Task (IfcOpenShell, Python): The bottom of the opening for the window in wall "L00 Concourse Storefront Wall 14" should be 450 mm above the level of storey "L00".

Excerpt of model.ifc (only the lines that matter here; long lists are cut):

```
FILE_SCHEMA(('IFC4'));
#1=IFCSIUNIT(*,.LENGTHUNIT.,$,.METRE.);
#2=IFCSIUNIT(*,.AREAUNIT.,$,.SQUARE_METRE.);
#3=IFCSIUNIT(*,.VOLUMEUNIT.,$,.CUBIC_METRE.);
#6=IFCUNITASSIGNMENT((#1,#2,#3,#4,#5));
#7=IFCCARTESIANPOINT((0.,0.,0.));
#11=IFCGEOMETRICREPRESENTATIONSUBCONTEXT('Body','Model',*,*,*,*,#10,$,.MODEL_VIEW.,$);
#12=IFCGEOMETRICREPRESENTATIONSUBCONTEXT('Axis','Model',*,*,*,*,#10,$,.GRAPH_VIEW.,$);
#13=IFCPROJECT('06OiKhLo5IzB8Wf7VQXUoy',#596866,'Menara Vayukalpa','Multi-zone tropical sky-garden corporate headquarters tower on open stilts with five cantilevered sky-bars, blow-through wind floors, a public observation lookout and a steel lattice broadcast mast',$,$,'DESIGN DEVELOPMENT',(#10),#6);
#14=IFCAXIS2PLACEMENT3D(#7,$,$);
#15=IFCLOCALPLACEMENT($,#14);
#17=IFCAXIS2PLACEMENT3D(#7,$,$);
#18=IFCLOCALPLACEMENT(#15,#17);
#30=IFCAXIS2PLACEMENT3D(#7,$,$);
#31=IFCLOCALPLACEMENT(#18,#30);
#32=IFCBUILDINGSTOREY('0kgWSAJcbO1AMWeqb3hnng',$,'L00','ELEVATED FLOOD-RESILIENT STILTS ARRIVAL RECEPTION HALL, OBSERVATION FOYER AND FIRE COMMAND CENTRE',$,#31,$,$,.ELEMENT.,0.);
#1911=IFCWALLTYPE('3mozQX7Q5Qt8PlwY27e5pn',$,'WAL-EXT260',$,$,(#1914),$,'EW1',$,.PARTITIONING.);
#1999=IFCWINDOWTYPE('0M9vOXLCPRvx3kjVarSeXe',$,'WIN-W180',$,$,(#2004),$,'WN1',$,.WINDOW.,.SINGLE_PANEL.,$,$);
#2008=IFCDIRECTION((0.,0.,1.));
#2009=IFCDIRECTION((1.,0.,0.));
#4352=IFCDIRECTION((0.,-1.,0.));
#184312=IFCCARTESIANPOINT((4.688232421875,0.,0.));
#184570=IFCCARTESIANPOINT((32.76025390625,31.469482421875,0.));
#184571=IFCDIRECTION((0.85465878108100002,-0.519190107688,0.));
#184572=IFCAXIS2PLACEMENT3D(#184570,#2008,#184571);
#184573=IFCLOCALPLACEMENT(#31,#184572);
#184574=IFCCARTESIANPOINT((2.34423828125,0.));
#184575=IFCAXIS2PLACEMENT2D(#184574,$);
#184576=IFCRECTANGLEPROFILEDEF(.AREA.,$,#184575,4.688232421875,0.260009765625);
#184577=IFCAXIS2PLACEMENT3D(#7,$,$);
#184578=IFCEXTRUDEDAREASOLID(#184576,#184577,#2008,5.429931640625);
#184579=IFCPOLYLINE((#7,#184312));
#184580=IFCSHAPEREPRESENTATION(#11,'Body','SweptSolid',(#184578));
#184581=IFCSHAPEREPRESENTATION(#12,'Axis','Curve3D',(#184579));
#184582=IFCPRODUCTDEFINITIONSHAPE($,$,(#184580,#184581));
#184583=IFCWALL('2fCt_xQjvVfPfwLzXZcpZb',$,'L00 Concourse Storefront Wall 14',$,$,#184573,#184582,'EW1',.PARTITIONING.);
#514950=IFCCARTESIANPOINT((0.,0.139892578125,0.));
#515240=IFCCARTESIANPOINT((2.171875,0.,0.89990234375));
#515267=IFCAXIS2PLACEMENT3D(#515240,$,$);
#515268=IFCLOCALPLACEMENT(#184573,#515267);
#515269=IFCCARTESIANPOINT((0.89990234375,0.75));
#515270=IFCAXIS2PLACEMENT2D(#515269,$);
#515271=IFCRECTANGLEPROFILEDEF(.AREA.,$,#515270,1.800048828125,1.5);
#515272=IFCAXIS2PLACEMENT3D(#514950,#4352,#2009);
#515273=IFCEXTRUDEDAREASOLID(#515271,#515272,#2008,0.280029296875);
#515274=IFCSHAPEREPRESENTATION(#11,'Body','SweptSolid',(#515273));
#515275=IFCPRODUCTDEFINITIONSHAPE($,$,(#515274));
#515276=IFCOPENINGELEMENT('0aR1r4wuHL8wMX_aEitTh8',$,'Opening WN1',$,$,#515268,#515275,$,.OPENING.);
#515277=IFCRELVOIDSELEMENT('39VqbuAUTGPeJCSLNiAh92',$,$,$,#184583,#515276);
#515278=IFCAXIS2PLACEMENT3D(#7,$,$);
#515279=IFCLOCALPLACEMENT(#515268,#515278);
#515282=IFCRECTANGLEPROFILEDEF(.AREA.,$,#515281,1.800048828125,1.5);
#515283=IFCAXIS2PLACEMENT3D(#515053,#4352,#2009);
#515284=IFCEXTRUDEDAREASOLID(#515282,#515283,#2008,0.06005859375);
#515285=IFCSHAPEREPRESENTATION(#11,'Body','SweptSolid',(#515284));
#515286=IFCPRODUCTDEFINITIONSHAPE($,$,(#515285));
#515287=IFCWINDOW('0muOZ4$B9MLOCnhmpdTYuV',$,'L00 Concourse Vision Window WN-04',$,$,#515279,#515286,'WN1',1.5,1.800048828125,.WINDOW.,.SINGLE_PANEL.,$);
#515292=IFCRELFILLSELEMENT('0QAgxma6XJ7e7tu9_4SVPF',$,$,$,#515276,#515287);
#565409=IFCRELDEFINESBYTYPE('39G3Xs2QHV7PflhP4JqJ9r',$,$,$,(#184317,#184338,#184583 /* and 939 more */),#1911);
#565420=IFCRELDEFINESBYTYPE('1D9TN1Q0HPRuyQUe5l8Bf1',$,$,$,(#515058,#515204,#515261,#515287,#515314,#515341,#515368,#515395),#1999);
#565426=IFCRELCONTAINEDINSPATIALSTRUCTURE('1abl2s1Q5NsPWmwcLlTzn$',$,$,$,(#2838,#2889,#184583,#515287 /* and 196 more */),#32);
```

```python
import numpy as np
import ifcopenshell
import ifcopenshell.api.geometry
import ifcopenshell.geom
import ifcopenshell.util.element
import ifcopenshell.util.placement
import ifcopenshell.util.shape
import ifcopenshell.util.unit

model = ifcopenshell.open("model.ifc")
unit_scale = ifcopenshell.util.unit.calculate_unit_scale(model)

window = model.by_guid("0muOZ4$B9MLOCnhmpdTYuV")
opening = window.FillsVoids[0].RelatingOpeningElement
storey = ifcopenshell.util.element.get_container(window, ifc_class="IfcBuildingStorey")
level = ifcopenshell.util.placement.get_local_placement(storey.ObjectPlacement)[2, 3]

# The opening's origin need not be at the sill, so measure its lowest point.
shape = ifcopenshell.geom.create_shape(ifcopenshell.geom.settings(), opening)
bottom = ifcopenshell.util.shape.get_shape_bottom_elevation(shape, shape.geometry) / unit_scale
dz = level + 0.45 - bottom

shift = np.array([0.0, 0.0, dz])
# The window is placed relative to its opening, so it follows when the opening moves.
matrix = ifcopenshell.util.placement.get_local_placement(opening.ObjectPlacement)
matrix[:3, 3] += shift
ifcopenshell.api.geometry.edit_object_placement(
    model, product=opening, matrix=matrix, is_si=False, should_transform_children=True
)

print(f"moved by {dz * unit_scale:+.3f} m")

model.write("model-out.ifc")
```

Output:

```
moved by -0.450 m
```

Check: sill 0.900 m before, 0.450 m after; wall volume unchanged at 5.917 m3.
